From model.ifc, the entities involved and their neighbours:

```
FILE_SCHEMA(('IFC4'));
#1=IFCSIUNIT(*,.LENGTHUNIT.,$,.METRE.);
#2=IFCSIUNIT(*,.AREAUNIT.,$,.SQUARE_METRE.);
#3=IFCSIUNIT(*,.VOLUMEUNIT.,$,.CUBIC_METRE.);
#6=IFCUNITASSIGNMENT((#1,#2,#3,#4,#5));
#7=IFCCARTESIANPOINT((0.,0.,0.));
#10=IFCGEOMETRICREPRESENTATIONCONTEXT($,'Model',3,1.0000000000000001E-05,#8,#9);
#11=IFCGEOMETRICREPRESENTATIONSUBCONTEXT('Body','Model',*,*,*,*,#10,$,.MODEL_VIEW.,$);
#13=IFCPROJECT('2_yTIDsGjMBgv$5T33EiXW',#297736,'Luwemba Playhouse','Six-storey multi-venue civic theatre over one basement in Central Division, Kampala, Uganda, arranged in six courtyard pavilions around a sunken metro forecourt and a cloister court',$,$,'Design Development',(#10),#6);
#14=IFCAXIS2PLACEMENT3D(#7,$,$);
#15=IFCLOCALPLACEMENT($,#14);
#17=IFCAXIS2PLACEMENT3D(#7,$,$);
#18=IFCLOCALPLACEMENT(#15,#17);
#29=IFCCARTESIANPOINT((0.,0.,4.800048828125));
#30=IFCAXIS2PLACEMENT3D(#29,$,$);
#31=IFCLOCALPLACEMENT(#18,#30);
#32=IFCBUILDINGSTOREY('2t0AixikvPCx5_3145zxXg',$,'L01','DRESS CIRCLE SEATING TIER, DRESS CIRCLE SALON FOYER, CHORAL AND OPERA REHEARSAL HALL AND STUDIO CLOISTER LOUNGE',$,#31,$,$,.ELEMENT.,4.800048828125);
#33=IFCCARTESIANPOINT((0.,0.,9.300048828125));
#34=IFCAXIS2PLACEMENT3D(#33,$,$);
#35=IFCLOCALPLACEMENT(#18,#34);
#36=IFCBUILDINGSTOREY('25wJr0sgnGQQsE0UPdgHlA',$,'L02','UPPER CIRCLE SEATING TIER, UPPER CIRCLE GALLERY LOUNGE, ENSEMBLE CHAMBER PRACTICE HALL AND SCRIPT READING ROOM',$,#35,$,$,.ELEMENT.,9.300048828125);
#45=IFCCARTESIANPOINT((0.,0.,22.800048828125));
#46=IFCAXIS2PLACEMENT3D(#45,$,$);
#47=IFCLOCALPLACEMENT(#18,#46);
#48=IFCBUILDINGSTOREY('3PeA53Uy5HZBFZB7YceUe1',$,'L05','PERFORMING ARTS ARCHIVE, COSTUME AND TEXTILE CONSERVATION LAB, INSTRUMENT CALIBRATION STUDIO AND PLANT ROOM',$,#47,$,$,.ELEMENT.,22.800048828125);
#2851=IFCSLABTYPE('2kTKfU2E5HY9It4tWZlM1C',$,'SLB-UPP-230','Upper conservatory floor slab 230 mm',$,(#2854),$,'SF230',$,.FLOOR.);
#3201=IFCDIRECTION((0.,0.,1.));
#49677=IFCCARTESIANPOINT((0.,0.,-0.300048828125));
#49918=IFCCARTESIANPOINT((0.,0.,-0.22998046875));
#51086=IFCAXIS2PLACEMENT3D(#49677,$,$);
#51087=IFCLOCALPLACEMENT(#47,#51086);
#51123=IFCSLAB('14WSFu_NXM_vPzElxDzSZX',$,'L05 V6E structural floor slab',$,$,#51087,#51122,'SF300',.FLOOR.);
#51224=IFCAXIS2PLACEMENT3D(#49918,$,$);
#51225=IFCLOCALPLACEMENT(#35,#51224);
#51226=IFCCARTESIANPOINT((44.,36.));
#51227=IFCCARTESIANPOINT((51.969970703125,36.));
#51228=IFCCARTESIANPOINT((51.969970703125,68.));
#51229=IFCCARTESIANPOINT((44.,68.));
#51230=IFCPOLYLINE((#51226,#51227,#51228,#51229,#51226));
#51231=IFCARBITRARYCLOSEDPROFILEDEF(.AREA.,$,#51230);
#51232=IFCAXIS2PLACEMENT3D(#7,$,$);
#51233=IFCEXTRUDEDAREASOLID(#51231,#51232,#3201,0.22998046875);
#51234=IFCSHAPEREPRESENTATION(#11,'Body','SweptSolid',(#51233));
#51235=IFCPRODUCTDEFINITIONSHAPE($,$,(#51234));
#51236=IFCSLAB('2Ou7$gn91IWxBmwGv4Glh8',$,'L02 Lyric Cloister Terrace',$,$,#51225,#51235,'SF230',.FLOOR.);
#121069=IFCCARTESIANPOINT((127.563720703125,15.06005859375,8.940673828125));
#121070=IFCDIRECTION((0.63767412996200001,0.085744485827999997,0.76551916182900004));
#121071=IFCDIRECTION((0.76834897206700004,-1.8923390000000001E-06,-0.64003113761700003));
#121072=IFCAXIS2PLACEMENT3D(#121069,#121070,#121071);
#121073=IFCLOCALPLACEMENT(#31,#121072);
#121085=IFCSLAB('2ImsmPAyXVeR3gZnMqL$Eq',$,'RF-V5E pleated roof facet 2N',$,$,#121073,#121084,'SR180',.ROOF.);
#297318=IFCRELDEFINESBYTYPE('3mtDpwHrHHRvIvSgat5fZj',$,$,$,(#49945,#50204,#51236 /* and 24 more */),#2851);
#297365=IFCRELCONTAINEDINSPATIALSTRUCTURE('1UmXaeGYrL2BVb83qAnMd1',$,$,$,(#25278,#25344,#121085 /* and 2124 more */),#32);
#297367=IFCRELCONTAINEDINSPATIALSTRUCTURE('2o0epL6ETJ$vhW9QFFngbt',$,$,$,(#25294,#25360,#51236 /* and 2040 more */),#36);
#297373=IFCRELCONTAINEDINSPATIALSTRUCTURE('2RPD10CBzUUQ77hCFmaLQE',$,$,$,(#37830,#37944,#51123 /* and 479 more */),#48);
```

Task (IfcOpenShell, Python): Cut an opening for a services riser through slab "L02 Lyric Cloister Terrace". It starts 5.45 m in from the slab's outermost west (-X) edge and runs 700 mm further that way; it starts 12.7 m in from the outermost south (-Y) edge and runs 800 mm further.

```python
import numpy as np
import ifcopenshell
import ifcopenshell.api.feature
import ifcopenshell.api.geometry
import ifcopenshell.api.root
import ifcopenshell.geom
import ifcopenshell.util.placement
import ifcopenshell.util.representation
import ifcopenshell.util.shape
import ifcopenshell.util.unit

model = ifcopenshell.open("model.ifc")
unit_scale = ifcopenshell.util.unit.calculate_unit_scale(model)
settings = ifcopenshell.geom.settings()


def volume(element):
    """Net volume in cubic metres, openings subtracted."""
    shape = ifcopenshell.geom.create_shape(settings, element)
    return ifcopenshell.util.shape.get_volume(shape.geometry)


slab = model.by_id(51236)
before = volume(slab)

# Extent in the slab's own axes, in metres. The edges named are its -X and -Y sides.
slab_shape = ifcopenshell.geom.create_shape(settings, slab)
vertices = ifcopenshell.util.shape.get_vertices(slab_shape.geometry)
x_min, y_min, bottom = vertices.min(axis=0)
top = vertices[:, 2].max()

opening = ifcopenshell.api.root.create_entity(model, ifc_class="IfcOpeningElement", name="Services riser opening", predefined_type="OPENING")
context = ifcopenshell.util.representation.get_context(model, "Model", "Body", "MODEL_VIEW")
width, depth = 0.7, 0.8
outline = [(0.0, 0.0), (width, 0.0), (width, depth), (0.0, depth), (0.0, 0.0)]
# Overshoot both faces by 50 mm so the cut is clean.
shape = ifcopenshell.api.geometry.add_slab_representation(
    model, context=context, depth=top - bottom + 0.1, polyline=outline
)
ifcopenshell.api.geometry.assign_representation(model, product=opening, representation=shape)

matrix = ifcopenshell.util.placement.get_local_placement(slab.ObjectPlacement)
matrix[:, 3] = matrix @ np.append(np.array([x_min + 5.45, y_min + 12.7, bottom - 0.05]) / unit_scale, 1.0)
ifcopenshell.api.geometry.edit_object_placement(model, product=opening, matrix=matrix, is_si=False)
ifcopenshell.api.feature.add_feature(model, feature=opening, element=slab)

after = volume(slab)

print(f"slab volume {before:.3f} -> {after:.3f} m3")

model.write("model-out.ifc")
```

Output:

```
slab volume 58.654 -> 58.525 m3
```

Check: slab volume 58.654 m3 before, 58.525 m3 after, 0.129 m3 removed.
